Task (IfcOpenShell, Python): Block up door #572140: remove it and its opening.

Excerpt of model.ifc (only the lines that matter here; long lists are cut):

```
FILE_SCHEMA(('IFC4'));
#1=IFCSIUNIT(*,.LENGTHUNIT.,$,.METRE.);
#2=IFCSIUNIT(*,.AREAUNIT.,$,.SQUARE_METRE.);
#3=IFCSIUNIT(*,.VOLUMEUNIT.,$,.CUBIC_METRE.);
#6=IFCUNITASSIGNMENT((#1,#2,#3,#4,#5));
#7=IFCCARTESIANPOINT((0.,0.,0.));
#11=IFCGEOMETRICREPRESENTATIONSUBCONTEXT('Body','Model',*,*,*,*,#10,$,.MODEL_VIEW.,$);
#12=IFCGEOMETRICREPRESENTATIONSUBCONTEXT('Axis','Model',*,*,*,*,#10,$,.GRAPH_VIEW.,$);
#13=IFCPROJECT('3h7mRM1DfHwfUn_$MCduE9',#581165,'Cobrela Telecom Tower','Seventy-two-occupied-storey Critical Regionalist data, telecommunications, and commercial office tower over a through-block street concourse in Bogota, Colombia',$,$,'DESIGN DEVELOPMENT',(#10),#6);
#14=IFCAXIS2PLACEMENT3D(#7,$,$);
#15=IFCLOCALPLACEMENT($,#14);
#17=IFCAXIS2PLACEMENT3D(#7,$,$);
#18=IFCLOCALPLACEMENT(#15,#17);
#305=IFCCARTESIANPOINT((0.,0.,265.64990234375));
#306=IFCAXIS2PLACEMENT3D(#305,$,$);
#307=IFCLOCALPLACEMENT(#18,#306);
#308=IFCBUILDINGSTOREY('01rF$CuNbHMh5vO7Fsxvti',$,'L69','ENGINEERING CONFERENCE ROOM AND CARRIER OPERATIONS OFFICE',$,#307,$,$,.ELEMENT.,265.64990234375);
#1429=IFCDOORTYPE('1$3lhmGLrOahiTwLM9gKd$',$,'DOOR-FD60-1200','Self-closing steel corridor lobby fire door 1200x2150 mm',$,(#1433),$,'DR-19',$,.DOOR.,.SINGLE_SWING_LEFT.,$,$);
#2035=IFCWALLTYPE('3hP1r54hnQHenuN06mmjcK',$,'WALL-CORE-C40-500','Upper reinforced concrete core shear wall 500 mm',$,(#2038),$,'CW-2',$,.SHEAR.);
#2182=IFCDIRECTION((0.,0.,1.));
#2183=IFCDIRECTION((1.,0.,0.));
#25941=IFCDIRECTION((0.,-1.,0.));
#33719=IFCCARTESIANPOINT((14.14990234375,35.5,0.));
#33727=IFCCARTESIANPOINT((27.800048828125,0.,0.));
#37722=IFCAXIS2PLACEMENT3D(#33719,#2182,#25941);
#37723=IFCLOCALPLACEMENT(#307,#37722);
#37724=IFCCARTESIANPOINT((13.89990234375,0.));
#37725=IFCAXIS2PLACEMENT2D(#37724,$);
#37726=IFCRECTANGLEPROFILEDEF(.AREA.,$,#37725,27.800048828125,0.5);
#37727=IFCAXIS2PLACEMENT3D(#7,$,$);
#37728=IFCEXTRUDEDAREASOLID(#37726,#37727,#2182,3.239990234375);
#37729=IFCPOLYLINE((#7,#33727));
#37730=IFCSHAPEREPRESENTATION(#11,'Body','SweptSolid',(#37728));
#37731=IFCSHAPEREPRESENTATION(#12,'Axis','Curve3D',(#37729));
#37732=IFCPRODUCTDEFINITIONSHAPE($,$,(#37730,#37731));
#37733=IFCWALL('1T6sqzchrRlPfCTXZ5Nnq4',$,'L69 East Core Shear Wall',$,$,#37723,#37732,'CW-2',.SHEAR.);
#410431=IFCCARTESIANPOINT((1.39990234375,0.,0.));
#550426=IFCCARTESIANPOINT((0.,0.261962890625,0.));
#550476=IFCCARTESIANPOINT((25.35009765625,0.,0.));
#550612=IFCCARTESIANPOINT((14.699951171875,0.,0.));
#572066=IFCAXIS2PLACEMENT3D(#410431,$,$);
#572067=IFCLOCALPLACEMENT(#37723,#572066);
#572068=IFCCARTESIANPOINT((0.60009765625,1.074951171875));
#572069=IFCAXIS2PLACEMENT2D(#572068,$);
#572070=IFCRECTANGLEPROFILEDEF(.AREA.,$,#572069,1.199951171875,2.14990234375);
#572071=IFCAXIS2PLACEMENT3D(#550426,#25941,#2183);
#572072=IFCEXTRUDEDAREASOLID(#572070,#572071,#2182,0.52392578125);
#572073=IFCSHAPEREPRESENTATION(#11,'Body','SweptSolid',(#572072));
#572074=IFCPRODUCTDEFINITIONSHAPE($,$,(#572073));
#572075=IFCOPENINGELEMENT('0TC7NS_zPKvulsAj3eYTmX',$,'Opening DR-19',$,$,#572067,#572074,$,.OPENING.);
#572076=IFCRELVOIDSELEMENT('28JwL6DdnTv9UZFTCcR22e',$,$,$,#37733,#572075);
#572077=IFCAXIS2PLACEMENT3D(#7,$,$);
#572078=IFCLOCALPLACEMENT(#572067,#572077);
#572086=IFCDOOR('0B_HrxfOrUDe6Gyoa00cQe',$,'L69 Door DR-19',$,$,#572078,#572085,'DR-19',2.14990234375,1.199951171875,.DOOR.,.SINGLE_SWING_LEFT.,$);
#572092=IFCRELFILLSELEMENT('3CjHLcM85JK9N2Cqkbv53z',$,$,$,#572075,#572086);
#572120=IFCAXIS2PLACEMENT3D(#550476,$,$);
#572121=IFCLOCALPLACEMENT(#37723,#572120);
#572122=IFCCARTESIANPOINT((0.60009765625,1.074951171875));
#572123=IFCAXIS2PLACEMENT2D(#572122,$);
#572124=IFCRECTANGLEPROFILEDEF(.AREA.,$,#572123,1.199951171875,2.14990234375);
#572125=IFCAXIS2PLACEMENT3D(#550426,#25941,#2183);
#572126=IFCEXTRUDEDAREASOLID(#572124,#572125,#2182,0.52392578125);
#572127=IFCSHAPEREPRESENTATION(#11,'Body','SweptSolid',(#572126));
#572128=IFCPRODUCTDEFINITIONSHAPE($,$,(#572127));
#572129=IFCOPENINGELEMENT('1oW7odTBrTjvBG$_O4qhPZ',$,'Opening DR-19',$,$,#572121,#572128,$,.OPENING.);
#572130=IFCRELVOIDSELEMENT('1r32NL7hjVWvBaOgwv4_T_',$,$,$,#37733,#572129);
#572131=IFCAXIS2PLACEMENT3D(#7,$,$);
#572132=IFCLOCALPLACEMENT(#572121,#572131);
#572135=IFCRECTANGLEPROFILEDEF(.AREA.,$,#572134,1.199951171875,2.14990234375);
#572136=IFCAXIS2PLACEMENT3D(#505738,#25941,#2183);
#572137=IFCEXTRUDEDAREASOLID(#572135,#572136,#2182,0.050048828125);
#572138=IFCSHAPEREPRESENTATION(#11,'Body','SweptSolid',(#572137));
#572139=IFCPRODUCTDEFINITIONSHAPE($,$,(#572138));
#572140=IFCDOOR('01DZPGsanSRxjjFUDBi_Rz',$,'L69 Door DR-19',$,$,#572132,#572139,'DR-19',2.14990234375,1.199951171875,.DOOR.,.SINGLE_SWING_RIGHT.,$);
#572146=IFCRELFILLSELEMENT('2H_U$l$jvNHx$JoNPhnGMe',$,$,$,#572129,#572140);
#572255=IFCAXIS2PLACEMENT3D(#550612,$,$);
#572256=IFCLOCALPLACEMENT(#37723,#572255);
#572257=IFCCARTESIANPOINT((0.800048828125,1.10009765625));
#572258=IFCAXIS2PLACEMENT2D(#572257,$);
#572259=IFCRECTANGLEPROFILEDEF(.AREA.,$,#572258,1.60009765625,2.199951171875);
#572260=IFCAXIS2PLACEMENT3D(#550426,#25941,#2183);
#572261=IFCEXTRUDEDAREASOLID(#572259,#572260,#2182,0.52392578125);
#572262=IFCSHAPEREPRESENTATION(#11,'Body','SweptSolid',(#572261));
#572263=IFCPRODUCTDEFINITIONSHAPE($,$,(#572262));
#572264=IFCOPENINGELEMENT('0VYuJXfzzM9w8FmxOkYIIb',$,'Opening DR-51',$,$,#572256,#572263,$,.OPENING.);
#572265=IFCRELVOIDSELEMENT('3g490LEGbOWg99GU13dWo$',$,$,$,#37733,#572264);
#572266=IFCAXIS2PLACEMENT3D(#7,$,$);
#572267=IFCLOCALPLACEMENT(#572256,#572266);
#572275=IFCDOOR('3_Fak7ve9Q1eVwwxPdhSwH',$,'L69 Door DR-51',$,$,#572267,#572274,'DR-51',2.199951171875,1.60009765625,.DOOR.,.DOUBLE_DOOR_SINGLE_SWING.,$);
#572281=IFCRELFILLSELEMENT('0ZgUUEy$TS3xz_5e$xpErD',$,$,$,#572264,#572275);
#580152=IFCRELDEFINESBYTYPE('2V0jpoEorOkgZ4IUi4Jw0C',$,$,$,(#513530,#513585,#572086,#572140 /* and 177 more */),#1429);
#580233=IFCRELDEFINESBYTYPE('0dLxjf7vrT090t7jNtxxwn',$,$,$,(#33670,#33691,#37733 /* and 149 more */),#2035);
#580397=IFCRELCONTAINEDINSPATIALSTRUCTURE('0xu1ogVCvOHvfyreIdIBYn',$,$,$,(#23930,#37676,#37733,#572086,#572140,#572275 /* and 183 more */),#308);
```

```python
import ifcopenshell
import ifcopenshell.api.feature
import ifcopenshell.api.root
import ifcopenshell.geom
import ifcopenshell.util.shape

model = ifcopenshell.open("model.ifc")
settings = ifcopenshell.geom.settings()


def volume(element):
    """Net volume in cubic metres, openings subtracted."""
    shape = ifcopenshell.geom.create_shape(settings, element)
    return ifcopenshell.util.shape.get_volume(shape.geometry)


door = model.by_id(572140)
opening = door.FillsVoids[0].RelatingOpeningElement
wall = opening.VoidsElements[0].RelatingBuildingElement
before = volume(wall)

ifcopenshell.api.root.remove_product(model, product=door)
ifcopenshell.api.feature.remove_feature(model, feature=opening)

after = volume(wall)

print(f"wall volume {before:.3f} -> {after:.3f} m3")

model.write("model_rev.ifc")
```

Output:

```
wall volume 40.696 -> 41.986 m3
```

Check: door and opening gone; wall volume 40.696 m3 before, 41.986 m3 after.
